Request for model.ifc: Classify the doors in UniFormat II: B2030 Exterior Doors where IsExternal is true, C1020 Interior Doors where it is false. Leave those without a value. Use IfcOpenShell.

First a look at what the model holds.

```python
import ifcopenshell
import ifcopenshell.util.element

model = ifcopenshell.open("model.ifc")
print(model.schema)
print("classifications:", [c.Name for c in model.by_type("IfcClassification")])
values = [ifcopenshell.util.element.get_pset(e, "Pset_DoorCommon", "IsExternal") for e in model.by_type("IfcDoor")]
for value in (True, False, None):
    print("IsExternal", value, values.count(value))
```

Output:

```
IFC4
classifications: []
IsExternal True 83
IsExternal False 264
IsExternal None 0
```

```python
import ifcopenshell
import ifcopenshell.api.classification
import ifcopenshell.util.element

model = ifcopenshell.open("model.ifc")

system = ifcopenshell.api.classification.add_classification(model, classification="UniFormat II")

doors = model.by_type("IfcDoor")
external = {e: ifcopenshell.util.element.get_pset(e, "Pset_DoorCommon", "IsExternal") for e in doors}
for flag, code, name in ((True, "B2030", "Exterior Doors"), (False, "C1020", "Interior Doors")):
    products = [e for e in doors if external[e] is flag]
    ifcopenshell.api.classification.add_reference(
        model, products=products, classification=system, identification=code, name=name
    )
    print(code, len(products))

model.write("model_rev.ifc")
```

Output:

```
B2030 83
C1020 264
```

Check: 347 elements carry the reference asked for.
